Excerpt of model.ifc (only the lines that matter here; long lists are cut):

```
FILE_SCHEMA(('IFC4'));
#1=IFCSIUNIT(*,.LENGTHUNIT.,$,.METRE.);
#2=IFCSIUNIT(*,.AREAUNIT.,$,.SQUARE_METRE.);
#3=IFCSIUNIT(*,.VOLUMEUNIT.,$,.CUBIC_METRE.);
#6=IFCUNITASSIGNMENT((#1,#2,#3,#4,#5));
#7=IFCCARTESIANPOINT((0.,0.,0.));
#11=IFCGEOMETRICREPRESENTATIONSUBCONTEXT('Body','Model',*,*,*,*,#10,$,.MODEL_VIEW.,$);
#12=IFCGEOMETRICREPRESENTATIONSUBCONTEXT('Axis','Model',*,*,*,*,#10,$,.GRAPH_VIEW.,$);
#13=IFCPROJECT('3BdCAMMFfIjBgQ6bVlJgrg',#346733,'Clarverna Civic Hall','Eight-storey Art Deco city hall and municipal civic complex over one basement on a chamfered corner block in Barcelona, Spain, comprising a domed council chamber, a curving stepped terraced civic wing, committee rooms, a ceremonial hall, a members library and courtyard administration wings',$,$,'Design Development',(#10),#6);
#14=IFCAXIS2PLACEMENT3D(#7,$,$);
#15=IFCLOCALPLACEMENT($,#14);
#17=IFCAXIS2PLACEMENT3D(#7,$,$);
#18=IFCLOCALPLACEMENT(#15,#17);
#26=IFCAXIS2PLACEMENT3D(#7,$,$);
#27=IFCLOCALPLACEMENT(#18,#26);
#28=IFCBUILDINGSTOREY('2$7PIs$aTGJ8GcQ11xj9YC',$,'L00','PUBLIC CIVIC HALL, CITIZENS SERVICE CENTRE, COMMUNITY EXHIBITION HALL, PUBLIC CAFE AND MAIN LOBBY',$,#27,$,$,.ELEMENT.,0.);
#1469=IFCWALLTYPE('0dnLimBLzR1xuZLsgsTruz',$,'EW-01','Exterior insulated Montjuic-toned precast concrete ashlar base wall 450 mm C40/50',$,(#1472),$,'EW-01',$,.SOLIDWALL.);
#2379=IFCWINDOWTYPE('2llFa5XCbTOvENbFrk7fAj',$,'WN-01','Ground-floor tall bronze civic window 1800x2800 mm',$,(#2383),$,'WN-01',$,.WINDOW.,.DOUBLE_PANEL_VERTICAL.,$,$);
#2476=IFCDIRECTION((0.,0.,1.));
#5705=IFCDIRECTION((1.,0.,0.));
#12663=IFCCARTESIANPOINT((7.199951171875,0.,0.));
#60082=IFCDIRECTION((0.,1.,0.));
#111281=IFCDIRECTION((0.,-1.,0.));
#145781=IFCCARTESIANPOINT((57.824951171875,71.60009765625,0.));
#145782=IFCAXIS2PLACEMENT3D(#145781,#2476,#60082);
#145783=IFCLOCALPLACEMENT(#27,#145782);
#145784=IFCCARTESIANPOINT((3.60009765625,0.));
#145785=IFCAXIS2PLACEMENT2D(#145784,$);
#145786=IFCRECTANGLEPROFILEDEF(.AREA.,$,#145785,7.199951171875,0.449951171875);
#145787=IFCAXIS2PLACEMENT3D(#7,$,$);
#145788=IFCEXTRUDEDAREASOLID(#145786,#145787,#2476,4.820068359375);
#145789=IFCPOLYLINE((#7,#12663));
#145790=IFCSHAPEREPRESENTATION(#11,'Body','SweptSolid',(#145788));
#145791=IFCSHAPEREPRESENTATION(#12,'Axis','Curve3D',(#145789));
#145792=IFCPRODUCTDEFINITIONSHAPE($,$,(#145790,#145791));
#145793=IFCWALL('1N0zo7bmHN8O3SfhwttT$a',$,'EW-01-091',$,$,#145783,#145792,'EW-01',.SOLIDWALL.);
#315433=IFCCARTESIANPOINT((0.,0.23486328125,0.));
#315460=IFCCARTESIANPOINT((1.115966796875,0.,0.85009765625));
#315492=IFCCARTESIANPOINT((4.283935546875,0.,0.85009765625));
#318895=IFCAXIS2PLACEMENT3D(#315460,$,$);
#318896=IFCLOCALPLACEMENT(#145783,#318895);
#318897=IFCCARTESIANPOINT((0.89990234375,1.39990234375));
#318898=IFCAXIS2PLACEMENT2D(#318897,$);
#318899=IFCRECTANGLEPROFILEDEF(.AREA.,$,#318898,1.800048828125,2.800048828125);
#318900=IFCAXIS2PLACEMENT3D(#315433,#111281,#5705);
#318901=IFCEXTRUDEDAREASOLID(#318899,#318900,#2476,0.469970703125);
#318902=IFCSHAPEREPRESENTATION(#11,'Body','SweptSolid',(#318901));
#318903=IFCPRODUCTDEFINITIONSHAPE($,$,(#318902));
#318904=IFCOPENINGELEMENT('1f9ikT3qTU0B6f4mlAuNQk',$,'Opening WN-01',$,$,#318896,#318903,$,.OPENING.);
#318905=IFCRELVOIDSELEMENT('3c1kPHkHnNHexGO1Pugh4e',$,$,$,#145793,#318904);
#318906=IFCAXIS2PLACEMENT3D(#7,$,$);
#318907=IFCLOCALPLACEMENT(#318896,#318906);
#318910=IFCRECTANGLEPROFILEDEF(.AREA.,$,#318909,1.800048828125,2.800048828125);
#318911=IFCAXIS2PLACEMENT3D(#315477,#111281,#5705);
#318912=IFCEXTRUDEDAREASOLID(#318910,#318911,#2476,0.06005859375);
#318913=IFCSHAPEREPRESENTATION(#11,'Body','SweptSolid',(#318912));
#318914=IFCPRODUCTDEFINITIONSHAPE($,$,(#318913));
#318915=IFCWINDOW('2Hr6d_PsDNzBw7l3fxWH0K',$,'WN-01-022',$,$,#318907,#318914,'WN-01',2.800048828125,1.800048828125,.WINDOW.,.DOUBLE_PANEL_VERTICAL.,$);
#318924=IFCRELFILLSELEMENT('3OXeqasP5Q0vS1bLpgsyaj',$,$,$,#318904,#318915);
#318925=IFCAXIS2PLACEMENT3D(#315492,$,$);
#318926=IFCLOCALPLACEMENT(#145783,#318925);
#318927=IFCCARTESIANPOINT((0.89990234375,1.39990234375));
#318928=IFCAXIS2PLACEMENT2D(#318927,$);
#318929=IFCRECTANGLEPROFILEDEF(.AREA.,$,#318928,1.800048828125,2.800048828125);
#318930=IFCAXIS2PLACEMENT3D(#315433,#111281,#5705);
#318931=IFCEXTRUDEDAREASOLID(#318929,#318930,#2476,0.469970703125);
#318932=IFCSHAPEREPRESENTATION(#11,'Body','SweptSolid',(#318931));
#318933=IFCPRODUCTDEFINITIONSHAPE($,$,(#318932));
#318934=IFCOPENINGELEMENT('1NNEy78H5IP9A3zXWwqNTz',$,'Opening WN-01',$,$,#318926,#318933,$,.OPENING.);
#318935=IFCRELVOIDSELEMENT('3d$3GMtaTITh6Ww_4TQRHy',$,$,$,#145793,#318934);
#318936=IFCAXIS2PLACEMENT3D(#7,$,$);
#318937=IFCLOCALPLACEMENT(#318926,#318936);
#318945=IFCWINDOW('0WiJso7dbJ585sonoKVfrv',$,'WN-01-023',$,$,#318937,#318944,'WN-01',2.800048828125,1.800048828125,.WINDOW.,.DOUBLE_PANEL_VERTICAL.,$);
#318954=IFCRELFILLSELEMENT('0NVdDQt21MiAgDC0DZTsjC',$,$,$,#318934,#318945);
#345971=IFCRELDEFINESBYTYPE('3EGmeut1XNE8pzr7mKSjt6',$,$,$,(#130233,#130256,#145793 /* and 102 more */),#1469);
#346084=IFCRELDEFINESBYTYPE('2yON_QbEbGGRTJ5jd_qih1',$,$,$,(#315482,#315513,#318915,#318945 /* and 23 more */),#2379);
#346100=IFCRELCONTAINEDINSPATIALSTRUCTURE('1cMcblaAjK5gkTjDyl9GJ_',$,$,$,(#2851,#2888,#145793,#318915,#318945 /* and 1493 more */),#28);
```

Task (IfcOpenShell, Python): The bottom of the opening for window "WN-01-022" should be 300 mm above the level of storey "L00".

```python
import numpy as np
import ifcopenshell
import ifcopenshell.api.geometry
import ifcopenshell.geom
import ifcopenshell.util.element
import ifcopenshell.util.placement
import ifcopenshell.util.shape
import ifcopenshell.util.unit

model = ifcopenshell.open("model.ifc")
unit_scale = ifcopenshell.util.unit.calculate_unit_scale(model)

window = model.by_id(318915)
opening = window.FillsVoids[0].RelatingOpeningElement
storey = ifcopenshell.util.element.get_container(window, ifc_class="IfcBuildingStorey")
level = ifcopenshell.util.placement.get_local_placement(storey.ObjectPlacement)[2, 3]

# The opening's origin need not be at the sill, so measure its lowest point.
shape = ifcopenshell.geom.create_shape(ifcopenshell.geom.settings(), opening)
bottom = ifcopenshell.util.shape.get_shape_bottom_elevation(shape, shape.geometry) / unit_scale
dz = level + 0.3 - bottom

shift = np.array([0.0, 0.0, dz])
# The window is placed relative to its opening, so it follows when the opening moves.
matrix = ifcopenshell.util.placement.get_local_placement(opening.ObjectPlacement)
matrix[:3, 3] += shift
ifcopenshell.api.geometry.edit_object_placement(
    model, product=opening, matrix=matrix, is_si=False, should_transform_children=True
)

print(f"moved by {dz * unit_scale:+.3f} m")

model.write("model_edited.ifc")
```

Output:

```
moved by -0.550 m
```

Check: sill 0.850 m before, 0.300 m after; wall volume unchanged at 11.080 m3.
